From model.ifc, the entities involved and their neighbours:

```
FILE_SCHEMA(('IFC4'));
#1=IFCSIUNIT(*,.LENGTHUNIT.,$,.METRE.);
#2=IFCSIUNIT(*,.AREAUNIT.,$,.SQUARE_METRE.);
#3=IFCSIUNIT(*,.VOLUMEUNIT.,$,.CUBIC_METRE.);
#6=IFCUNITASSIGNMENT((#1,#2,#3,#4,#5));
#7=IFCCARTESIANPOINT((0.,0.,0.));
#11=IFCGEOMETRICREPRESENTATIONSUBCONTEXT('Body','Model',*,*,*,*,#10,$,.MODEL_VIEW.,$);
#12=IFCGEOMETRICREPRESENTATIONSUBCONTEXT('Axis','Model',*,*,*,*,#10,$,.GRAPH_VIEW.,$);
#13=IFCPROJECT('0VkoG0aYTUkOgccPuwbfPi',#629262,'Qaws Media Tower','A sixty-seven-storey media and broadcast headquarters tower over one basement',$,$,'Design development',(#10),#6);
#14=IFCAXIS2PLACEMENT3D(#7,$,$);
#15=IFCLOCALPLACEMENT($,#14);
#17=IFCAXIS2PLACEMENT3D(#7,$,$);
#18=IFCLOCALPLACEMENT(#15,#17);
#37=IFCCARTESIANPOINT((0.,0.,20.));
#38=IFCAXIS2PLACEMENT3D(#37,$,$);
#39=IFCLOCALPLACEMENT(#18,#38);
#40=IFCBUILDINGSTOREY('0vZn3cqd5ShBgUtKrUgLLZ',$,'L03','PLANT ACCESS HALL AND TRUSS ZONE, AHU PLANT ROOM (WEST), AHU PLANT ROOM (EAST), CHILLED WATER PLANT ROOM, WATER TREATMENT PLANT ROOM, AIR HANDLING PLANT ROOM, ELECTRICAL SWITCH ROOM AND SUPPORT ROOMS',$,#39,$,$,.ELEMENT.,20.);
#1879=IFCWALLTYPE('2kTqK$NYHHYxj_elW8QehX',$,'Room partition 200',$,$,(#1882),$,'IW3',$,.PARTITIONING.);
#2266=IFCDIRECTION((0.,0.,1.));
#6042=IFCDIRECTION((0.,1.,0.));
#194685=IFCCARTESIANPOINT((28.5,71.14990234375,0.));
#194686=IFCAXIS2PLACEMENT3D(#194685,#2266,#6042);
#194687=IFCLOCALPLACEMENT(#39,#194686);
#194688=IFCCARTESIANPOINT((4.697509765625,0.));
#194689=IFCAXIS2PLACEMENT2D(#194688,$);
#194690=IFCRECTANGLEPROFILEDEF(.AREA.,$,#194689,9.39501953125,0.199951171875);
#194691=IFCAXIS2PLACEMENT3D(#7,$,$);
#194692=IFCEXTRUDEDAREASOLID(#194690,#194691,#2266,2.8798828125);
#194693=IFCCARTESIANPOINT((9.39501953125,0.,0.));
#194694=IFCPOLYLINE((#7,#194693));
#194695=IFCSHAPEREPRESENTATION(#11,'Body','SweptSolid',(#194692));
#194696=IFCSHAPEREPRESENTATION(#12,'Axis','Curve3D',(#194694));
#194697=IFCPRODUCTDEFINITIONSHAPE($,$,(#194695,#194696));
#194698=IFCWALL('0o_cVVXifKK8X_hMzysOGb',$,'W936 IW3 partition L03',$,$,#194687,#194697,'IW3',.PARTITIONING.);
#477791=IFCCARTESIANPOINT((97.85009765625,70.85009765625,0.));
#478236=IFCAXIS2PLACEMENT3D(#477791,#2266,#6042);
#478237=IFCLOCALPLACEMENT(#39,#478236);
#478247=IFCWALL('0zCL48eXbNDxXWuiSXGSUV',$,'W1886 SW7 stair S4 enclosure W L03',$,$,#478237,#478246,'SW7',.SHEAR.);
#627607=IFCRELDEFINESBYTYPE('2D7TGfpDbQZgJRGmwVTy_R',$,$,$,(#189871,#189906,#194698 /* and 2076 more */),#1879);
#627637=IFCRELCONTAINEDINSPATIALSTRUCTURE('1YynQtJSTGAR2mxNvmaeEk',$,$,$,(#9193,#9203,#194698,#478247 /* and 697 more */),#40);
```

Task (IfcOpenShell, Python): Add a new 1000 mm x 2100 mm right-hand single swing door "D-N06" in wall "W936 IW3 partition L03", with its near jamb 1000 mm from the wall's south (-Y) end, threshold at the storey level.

```python
import numpy as np
import ifcopenshell
import ifcopenshell.api.feature
import ifcopenshell.api.geometry
import ifcopenshell.api.root
import ifcopenshell.api.spatial
import ifcopenshell.geom
import ifcopenshell.util.element
import ifcopenshell.util.placement
import ifcopenshell.util.representation
import ifcopenshell.util.shape
import ifcopenshell.util.unit

model = ifcopenshell.open("model.ifc")
unit_scale = ifcopenshell.util.unit.calculate_unit_scale(model)
settings = ifcopenshell.geom.settings()


def volume(element):
    """Net volume in cubic metres, openings subtracted."""
    shape = ifcopenshell.geom.create_shape(settings, element)
    return ifcopenshell.util.shape.get_volume(shape.geometry)


wall = model.by_guid("0o_cVVXifKK8X_hMzysOGb")
storey = ifcopenshell.util.element.get_container(wall, ifc_class="IfcBuildingStorey")
context = ifcopenshell.util.representation.get_context(model, "Model", "Body", "MODEL_VIEW")
before = volume(wall)

width, height, from_end, sill = 1, 2.1, 1, 0.0  # metres

# The wall runs along its own X axis, and the end named is its -X end.
wall_shape = ifcopenshell.geom.create_shape(settings, wall)
x, y, z = ifcopenshell.util.shape.get_vertices(wall_shape.geometry).T
start = x.min() + from_end
face, thickness = float(y.min()), float(y.max() - y.min())
wall_matrix = ifcopenshell.util.placement.get_local_placement(wall.ObjectPlacement)
level = ifcopenshell.util.placement.get_local_placement(storey.ObjectPlacement)[2, 3]


def in_wall(x, y):
    """Placement at x, y metres in the wall's axes, at sill height."""
    matrix = wall_matrix.copy()
    matrix[:, 3] = wall_matrix @ np.array([x / unit_scale, y / unit_scale, 0.0, 1.0])
    matrix[2, 3] = level + sill / unit_scale
    return matrix


# Opening: a box that overshoots both wall faces by 50 mm.
opening = ifcopenshell.api.root.create_entity(model, ifc_class="IfcOpeningElement", predefined_type="OPENING")
box = ifcopenshell.api.geometry.add_wall_representation(
    model, context=context, length=width, height=height, thickness=thickness + 0.1
)
ifcopenshell.api.geometry.assign_representation(model, product=opening, representation=box)
ifcopenshell.api.geometry.edit_object_placement(model, product=opening, matrix=in_wall(start, face - 0.05), is_si=False)
ifcopenshell.api.feature.add_feature(model, feature=opening, element=wall)

door = ifcopenshell.api.root.create_entity(model, ifc_class="IfcDoor", name="D-N06", predefined_type="DOOR")
door.OverallWidth, door.OverallHeight = width / unit_scale, height / unit_scale
door.OperationType = "SINGLE_SWING_RIGHT"
body = ifcopenshell.api.geometry.add_door_representation(
    model,
    context=context,
    overall_width=door.OverallWidth,
    overall_height=door.OverallHeight,
    operation_type="SINGLE_SWING_RIGHT",
    lining_properties={"LiningDepth": thickness / unit_scale, "ThresholdDepth": thickness / unit_scale},
)
ifcopenshell.api.geometry.assign_representation(model, product=door, representation=body)
ifcopenshell.api.spatial.assign_container(model, products=[door], relating_structure=storey)
ifcopenshell.api.feature.add_filling(model, opening=opening, element=door)

# The lining spans the wall, so the door starts at the wall face.
ifcopenshell.api.geometry.edit_object_placement(model, product=door, matrix=in_wall(start, face), is_si=False)

after = volume(wall)

print(f"wall volume {before:.3f} -> {after:.3f} m3")

model.write("model_rev.ifc")
```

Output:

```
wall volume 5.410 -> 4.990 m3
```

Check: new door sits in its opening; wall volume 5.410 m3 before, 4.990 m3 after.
